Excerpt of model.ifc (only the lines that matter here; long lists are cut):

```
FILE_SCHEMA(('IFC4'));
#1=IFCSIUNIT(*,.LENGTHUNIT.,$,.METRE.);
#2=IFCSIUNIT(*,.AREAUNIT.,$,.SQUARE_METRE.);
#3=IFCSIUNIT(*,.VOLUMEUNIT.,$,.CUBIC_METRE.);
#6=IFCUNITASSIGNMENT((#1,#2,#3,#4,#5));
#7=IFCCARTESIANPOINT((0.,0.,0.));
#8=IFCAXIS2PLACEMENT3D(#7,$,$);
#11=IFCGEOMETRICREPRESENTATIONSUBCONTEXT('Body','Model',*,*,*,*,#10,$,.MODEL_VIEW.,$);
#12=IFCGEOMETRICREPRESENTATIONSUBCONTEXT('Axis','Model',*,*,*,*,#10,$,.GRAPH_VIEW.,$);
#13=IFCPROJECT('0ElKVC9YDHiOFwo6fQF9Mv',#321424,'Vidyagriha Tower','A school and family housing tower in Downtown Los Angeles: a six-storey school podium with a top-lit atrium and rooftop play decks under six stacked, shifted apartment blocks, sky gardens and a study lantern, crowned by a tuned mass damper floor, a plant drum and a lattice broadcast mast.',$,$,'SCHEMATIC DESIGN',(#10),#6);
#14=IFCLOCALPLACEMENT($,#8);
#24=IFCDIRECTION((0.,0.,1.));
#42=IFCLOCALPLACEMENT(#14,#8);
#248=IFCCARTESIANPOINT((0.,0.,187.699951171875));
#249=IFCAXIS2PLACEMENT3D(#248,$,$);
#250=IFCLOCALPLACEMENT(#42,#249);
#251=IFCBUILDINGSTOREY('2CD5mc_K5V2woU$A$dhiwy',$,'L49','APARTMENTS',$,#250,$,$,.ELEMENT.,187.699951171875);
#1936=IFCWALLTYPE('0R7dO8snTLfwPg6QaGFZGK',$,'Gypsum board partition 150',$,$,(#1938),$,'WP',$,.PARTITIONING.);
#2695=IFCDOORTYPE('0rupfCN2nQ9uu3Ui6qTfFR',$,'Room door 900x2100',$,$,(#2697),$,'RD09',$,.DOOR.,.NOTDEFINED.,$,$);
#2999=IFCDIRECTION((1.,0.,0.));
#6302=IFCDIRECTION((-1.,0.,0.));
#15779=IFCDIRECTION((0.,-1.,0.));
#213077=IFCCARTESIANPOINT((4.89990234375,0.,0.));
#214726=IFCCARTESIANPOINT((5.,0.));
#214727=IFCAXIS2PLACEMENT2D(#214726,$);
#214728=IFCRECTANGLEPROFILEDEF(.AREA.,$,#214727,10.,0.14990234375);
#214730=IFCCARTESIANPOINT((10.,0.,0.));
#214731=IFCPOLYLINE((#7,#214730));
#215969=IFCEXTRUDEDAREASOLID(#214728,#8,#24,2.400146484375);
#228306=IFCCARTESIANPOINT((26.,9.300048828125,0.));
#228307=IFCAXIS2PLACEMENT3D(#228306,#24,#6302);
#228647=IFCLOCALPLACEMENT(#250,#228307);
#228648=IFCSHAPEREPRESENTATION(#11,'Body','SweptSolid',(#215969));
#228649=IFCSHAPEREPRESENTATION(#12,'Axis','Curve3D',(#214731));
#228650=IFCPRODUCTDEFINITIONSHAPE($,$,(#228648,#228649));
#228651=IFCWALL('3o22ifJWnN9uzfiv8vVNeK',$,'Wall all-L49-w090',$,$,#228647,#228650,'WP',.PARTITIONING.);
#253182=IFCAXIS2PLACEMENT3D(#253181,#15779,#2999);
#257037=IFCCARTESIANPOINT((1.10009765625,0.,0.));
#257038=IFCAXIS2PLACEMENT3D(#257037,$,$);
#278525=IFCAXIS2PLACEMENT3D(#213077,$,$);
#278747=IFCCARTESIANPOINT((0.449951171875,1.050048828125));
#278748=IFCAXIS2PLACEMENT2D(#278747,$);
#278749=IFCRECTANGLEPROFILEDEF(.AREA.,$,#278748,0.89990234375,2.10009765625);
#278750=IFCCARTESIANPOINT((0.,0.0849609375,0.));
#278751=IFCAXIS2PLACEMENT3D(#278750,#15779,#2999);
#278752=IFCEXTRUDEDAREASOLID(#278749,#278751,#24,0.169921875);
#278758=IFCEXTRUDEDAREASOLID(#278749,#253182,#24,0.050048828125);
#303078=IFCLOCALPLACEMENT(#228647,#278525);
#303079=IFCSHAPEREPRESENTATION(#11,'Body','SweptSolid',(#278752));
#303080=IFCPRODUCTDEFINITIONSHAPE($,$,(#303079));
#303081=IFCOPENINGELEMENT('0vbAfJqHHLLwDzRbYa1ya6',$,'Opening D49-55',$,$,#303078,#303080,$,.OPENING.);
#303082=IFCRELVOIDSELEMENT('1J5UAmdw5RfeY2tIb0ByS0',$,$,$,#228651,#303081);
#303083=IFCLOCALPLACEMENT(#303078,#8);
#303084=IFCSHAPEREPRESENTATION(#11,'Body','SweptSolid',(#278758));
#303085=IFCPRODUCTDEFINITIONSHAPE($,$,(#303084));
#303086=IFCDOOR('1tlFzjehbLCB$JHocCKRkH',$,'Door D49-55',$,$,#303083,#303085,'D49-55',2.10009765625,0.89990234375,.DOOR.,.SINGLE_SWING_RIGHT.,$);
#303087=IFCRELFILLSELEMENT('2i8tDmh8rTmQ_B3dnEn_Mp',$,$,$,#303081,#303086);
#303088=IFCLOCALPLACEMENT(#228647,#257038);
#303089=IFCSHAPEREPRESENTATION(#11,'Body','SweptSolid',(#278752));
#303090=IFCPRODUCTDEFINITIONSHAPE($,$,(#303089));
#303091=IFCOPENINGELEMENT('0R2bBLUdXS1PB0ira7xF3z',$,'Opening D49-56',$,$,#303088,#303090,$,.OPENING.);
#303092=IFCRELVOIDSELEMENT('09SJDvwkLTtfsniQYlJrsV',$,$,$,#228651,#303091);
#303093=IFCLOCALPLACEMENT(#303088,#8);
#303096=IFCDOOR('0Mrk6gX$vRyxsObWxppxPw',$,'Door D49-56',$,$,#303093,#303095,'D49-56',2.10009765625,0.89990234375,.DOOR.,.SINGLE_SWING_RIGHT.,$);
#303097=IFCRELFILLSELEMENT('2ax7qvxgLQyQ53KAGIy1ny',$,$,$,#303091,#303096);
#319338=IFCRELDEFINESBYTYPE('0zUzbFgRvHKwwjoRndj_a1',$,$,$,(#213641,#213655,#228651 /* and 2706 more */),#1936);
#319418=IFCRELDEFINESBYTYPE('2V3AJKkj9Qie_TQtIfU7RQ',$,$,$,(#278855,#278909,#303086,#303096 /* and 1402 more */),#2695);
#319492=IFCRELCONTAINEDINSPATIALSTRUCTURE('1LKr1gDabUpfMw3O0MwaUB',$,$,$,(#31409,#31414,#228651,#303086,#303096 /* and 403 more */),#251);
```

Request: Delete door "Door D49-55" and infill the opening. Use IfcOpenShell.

```python
import ifcopenshell
import ifcopenshell.api.feature
import ifcopenshell.api.root
import ifcopenshell.geom
import ifcopenshell.util.shape

model = ifcopenshell.open("model.ifc")
settings = ifcopenshell.geom.settings()


def volume(element):
    """Net volume in cubic metres, openings subtracted."""
    shape = ifcopenshell.geom.create_shape(settings, element)
    return ifcopenshell.util.shape.get_volume(shape.geometry)


door = model.by_guid("1tlFzjehbLCB$JHocCKRkH")
opening = door.FillsVoids[0].RelatingOpeningElement
wall = opening.VoidsElements[0].RelatingBuildingElement
before = volume(wall)

ifcopenshell.api.root.remove_product(model, product=door)
ifcopenshell.api.feature.remove_feature(model, feature=opening)

after = volume(wall)

print(f"wall volume {before:.3f} -> {after:.3f} m3")

model.write("model_updated.ifc")
```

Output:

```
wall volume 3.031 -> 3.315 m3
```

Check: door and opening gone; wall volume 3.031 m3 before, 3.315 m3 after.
